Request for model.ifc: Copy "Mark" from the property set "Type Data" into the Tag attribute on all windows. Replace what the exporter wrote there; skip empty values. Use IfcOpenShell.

First a look at what the model holds.

```python
import ifcopenshell
import ifcopenshell.util.element

model = ifcopenshell.open("model.ifc")
print(model.schema)
windows = model.by_type("IfcWindow")
print(len(windows), "windows")
for e in windows[:8]:
    source = ifcopenshell.util.element.get_pset(e, "Type Data", "Mark")
    target = e.Tag
    print(e.id(), repr(source), repr(target), sep=" | ")
```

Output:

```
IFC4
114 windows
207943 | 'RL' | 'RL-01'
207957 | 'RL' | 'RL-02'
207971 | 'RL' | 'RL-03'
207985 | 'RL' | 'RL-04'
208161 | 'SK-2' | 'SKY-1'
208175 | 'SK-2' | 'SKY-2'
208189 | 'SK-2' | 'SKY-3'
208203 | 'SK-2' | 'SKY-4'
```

```python
import ifcopenshell
import ifcopenshell.util.element

model = ifcopenshell.open("model.ifc")

count = 0
for e in model.by_type("IfcWindow"):
    value = ifcopenshell.util.element.get_pset(e, "Type Data", "Mark")
    current = e.Tag
    if not value or not value.strip() or current == value:
        continue
    e.Tag = value
    count += 1

print(count, "windows updated")

model.write("model_updated.ifc")
```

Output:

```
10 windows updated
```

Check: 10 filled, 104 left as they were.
